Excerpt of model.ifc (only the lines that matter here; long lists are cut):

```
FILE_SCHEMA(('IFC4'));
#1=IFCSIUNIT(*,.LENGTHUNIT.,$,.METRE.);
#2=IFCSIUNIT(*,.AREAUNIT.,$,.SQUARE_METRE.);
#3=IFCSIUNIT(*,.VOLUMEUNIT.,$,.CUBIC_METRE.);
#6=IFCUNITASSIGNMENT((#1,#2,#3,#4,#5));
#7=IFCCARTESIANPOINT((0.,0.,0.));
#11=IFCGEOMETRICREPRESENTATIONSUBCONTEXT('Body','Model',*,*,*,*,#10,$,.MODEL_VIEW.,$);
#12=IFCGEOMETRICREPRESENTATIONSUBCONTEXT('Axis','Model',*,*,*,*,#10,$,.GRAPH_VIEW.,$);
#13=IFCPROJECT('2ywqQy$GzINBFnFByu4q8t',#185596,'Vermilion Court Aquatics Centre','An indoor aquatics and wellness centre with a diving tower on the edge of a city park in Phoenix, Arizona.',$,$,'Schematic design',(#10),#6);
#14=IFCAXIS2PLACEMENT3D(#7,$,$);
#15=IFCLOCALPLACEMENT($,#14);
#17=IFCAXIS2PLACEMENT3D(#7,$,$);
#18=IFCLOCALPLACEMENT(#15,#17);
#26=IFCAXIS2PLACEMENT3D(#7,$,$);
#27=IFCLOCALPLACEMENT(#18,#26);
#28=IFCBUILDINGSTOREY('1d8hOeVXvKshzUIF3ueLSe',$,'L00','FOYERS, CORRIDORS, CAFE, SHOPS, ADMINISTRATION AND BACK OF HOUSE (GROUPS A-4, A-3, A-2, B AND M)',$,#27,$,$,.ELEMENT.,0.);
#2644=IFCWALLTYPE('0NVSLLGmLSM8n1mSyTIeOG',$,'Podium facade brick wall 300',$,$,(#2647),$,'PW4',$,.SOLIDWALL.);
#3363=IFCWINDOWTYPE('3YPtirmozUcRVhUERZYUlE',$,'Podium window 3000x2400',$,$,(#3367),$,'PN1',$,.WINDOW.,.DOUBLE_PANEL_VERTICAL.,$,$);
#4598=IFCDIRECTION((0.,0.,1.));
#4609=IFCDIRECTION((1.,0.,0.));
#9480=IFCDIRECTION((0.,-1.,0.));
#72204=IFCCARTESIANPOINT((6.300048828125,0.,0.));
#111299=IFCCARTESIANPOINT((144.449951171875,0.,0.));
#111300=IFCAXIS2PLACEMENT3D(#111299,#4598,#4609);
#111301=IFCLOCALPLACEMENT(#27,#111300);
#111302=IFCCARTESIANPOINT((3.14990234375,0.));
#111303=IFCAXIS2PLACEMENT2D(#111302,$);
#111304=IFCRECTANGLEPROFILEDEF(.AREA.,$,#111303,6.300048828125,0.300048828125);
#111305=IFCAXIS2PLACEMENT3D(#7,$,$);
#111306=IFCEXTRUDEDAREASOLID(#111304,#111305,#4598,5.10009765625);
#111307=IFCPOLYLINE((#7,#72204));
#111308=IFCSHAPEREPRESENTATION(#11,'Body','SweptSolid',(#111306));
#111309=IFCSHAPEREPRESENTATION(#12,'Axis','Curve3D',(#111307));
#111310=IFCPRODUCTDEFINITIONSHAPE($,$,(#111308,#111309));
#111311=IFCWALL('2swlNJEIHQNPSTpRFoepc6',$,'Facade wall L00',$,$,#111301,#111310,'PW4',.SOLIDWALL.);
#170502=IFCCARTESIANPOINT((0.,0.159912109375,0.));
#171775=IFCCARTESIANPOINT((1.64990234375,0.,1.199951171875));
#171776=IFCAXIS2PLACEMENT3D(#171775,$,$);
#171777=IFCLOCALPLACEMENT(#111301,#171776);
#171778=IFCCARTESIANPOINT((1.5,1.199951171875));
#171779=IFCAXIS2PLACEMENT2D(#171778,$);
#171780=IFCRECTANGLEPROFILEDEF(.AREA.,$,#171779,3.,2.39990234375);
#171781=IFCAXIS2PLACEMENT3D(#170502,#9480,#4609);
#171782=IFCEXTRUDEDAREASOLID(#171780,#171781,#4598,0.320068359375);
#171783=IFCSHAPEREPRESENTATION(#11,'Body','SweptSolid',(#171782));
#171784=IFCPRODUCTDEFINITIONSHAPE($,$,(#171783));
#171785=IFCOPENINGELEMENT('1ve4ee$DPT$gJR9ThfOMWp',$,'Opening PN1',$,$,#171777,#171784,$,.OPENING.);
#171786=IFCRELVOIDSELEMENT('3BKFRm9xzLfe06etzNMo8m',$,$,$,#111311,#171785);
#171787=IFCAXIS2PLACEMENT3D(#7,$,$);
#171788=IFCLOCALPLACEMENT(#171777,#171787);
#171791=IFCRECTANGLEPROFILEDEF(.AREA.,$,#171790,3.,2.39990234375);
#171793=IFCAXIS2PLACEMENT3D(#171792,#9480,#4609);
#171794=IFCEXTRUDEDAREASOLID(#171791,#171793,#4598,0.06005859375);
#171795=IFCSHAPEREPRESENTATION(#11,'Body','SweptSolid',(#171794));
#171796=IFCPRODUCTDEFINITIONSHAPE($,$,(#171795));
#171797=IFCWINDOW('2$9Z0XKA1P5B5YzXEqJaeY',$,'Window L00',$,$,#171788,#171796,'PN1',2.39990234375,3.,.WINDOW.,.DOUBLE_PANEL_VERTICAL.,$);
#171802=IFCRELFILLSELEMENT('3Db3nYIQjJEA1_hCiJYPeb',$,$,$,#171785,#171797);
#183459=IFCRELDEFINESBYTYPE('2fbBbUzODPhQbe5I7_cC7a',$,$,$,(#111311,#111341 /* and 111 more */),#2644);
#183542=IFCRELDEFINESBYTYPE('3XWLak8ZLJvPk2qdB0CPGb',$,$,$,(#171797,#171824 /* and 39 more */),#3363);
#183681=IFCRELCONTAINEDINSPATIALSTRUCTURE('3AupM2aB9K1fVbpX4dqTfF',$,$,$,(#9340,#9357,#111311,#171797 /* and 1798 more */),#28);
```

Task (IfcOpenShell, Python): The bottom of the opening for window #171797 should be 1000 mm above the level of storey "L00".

```python
import numpy as np
import ifcopenshell
import ifcopenshell.api.geometry
import ifcopenshell.geom
import ifcopenshell.util.element
import ifcopenshell.util.placement
import ifcopenshell.util.shape
import ifcopenshell.util.unit

model = ifcopenshell.open("model.ifc")
unit_scale = ifcopenshell.util.unit.calculate_unit_scale(model)

window = model.by_guid("2$9Z0XKA1P5B5YzXEqJaeY")
opening = window.FillsVoids[0].RelatingOpeningElement
storey = ifcopenshell.util.element.get_container(window, ifc_class="IfcBuildingStorey")
level = ifcopenshell.util.placement.get_local_placement(storey.ObjectPlacement)[2, 3]

# The opening's origin need not be at the sill, so measure its lowest point.
shape = ifcopenshell.geom.create_shape(ifcopenshell.geom.settings(), opening)
bottom = ifcopenshell.util.shape.get_shape_bottom_elevation(shape, shape.geometry) / unit_scale
dz = level + 1 / unit_scale - bottom

shift = np.array([0.0, 0.0, dz])
# The window is placed relative to its opening, so it follows when the opening moves.
matrix = ifcopenshell.util.placement.get_local_placement(opening.ObjectPlacement)
matrix[:3, 3] += shift
ifcopenshell.api.geometry.edit_object_placement(
    model, product=opening, matrix=matrix, is_si=False, should_transform_children=True
)

print(f"moved by {dz * unit_scale:+.3f} m")

model.write("model_v2.ifc")
```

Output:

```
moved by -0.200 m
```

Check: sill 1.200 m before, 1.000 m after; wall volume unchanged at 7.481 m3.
